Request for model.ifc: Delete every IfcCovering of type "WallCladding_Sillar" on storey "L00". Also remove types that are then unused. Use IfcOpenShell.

First a look at what the model holds.

```python
import ifcopenshell
import ifcopenshell.util.element

model = ifcopenshell.open("model.ifc")
print(model.schema)
storey = next(s for s in model.by_type("IfcBuildingStorey") if s.Name == "L00")
coverings = [e for e in ifcopenshell.util.element.get_decomposition(storey) if e.is_a("IfcCovering")]
seen = {}
for e in coverings:
    element_type = ifcopenshell.util.element.get_type(e)
    name = element_type.Name if element_type not in (None, e) else None
    seen[name] = seen.get(name, 0) + 1
for name, count in sorted(seen.items(), key=str):
    print(count, "x", name)
```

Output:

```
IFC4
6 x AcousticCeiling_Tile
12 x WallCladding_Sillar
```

```python
import ifcopenshell
import ifcopenshell.api.root
import ifcopenshell.util.element

model = ifcopenshell.open("model.ifc")

storey = next(s for s in model.by_type("IfcBuildingStorey") if s.Name == "L00")
coverings = [e for e in ifcopenshell.util.element.get_decomposition(storey) if e.is_a("IfcCovering")]
targets = [e for e in coverings if (t := ifcopenshell.util.element.get_type(e)) not in (None, e) and t.Name == "WallCladding_Sillar"]
types = {ifcopenshell.util.element.get_type(e) for e in targets} - {None, *targets}

for e in targets:
    ifcopenshell.api.root.remove_product(model, product=e)
print(len(targets), "removed")

unused = [t for t in types if not ifcopenshell.util.element.get_types(t)]
for t in unused:
    ifcopenshell.api.root.remove_product(model, product=t)
print(len(unused), "unused types removed")

model.write("model-out.ifc")
```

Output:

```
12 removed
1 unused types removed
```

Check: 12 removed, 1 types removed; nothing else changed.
